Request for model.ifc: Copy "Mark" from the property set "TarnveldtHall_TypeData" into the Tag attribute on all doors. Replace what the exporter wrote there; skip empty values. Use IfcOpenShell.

First a look at what the model holds.

```python
import ifcopenshell
import ifcopenshell.util.element

model = ifcopenshell.open("model.ifc")
print(model.schema)
doors = model.by_type("IfcDoor")
print(len(doors), "doors")
for e in doors[:8]:
    source = ifcopenshell.util.element.get_pset(e, "TarnveldtHall_TypeData", "Mark")
    target = e.Tag
    print(e.id(), repr(source), repr(target), sep=" | ")
```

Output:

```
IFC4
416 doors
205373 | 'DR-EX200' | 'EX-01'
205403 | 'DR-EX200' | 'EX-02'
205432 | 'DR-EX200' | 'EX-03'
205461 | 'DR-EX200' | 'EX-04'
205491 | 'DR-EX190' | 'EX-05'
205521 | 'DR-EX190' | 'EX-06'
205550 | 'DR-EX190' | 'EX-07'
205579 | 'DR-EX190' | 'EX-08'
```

```python
import ifcopenshell
import ifcopenshell.util.element

model = ifcopenshell.open("model.ifc")

count = 0
for e in model.by_type("IfcDoor"):
    value = ifcopenshell.util.element.get_pset(e, "TarnveldtHall_TypeData", "Mark")
    current = e.Tag
    if not value or not value.strip() or current == value:
        continue
    e.Tag = value
    count += 1

print(count, "doors updated")

model.write("model_updated.ifc")
```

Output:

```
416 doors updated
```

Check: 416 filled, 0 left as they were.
